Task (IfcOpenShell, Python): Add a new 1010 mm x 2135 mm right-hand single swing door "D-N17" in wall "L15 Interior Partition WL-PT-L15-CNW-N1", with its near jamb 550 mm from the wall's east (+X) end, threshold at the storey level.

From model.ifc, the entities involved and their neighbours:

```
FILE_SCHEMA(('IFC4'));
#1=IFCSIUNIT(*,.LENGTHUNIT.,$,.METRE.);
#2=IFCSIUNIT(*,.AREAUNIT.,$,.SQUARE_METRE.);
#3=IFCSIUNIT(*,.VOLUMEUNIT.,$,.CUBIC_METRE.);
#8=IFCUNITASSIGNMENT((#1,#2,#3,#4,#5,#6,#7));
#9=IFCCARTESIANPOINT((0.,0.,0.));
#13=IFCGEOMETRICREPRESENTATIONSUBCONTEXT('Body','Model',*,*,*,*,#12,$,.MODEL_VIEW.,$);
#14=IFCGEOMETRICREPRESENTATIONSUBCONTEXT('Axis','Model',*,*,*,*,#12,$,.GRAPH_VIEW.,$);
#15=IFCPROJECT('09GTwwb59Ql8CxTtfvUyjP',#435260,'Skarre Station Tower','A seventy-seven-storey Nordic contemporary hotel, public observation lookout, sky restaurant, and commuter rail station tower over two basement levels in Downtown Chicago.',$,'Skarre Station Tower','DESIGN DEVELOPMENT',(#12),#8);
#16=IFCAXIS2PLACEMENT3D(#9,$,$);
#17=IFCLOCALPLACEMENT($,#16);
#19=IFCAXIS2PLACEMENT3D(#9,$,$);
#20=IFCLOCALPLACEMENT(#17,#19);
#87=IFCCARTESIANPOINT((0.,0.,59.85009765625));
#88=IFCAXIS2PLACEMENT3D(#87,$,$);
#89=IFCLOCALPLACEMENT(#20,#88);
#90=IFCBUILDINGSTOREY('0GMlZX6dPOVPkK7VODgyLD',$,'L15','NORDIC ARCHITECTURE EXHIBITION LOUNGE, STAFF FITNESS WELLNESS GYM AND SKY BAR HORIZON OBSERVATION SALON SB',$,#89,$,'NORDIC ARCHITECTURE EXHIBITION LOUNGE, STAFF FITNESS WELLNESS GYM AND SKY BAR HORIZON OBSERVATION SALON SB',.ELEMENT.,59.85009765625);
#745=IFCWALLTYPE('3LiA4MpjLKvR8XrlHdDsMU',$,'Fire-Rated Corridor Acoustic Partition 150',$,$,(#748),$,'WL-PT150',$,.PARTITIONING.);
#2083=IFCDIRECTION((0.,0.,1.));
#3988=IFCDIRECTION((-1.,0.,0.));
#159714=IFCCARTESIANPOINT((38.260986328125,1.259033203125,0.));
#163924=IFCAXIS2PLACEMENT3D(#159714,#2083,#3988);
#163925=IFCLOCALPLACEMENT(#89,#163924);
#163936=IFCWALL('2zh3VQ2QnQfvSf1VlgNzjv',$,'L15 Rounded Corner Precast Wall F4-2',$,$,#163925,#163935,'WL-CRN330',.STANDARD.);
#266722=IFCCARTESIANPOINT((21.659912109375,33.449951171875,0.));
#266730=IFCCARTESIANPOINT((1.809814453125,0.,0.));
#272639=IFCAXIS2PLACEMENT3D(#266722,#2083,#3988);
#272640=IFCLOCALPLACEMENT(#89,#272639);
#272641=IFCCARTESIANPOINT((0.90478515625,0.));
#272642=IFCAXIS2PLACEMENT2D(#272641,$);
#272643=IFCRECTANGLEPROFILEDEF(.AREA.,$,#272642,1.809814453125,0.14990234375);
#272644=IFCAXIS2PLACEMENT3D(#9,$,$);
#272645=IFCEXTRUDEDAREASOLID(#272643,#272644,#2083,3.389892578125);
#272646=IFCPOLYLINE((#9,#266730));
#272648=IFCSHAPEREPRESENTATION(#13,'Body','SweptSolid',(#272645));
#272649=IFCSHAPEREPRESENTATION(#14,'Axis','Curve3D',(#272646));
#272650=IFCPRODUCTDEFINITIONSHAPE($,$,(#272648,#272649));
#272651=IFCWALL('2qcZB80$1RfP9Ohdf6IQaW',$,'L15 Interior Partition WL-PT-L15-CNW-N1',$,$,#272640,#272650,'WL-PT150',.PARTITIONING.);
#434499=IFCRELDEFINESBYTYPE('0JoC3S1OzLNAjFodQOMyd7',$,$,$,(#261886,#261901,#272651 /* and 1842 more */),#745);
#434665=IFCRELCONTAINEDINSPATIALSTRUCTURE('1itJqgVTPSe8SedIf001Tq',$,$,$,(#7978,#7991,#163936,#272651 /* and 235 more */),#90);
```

```python
import numpy as np
import ifcopenshell
import ifcopenshell.api.feature
import ifcopenshell.api.geometry
import ifcopenshell.api.root
import ifcopenshell.api.spatial
import ifcopenshell.geom
import ifcopenshell.util.element
import ifcopenshell.util.placement
import ifcopenshell.util.representation
import ifcopenshell.util.shape
import ifcopenshell.util.unit

model = ifcopenshell.open("model.ifc")
unit_scale = ifcopenshell.util.unit.calculate_unit_scale(model)
settings = ifcopenshell.geom.settings()


def volume(element):
    """Net volume in cubic metres, openings subtracted."""
    shape = ifcopenshell.geom.create_shape(settings, element)
    return ifcopenshell.util.shape.get_volume(shape.geometry)


wall = model.by_guid("2qcZB80$1RfP9Ohdf6IQaW")
storey = ifcopenshell.util.element.get_container(wall, ifc_class="IfcBuildingStorey")
context = ifcopenshell.util.representation.get_context(model, "Model", "Body", "MODEL_VIEW")
before = volume(wall)

width, height, from_end, sill = 1.01, 2.135, 0.55, 0.0  # metres

# The wall runs along its own X axis, and the end named is its -X end.
wall_shape = ifcopenshell.geom.create_shape(settings, wall)
x, y, z = ifcopenshell.util.shape.get_vertices(wall_shape.geometry).T
start = x.min() + from_end
face, thickness = float(y.min()), float(y.max() - y.min())
wall_matrix = ifcopenshell.util.placement.get_local_placement(wall.ObjectPlacement)
level = ifcopenshell.util.placement.get_local_placement(storey.ObjectPlacement)[2, 3]


def in_wall(x, y):
    """Placement at x, y metres in the wall's axes, at sill height."""
    matrix = wall_matrix.copy()
    matrix[:, 3] = wall_matrix @ np.array([x / unit_scale, y / unit_scale, 0.0, 1.0])
    matrix[2, 3] = level + sill / unit_scale
    return matrix


# Opening: a box that overshoots both wall faces by 50 mm.
opening = ifcopenshell.api.root.create_entity(model, ifc_class="IfcOpeningElement", predefined_type="OPENING")
box = ifcopenshell.api.geometry.add_wall_representation(
    model, context=context, length=width, height=height, thickness=thickness + 0.1
)
ifcopenshell.api.geometry.assign_representation(model, product=opening, representation=box)
ifcopenshell.api.geometry.edit_object_placement(model, product=opening, matrix=in_wall(start, face - 0.05), is_si=False)
ifcopenshell.api.feature.add_feature(model, feature=opening, element=wall)

door = ifcopenshell.api.root.create_entity(model, ifc_class="IfcDoor", name="D-N17", predefined_type="DOOR")
door.OverallWidth, door.OverallHeight = width / unit_scale, height / unit_scale
door.OperationType = "SINGLE_SWING_RIGHT"
body = ifcopenshell.api.geometry.add_door_representation(
    model,
    context=context,
    overall_width=door.OverallWidth,
    overall_height=door.OverallHeight,
    operation_type="SINGLE_SWING_RIGHT",
    lining_properties={"LiningDepth": thickness / unit_scale, "ThresholdDepth": thickness / unit_scale},
)
ifcopenshell.api.geometry.assign_representation(model, product=door, representation=body)
ifcopenshell.api.spatial.assign_container(model, products=[door], relating_structure=storey)
ifcopenshell.api.feature.add_filling(model, opening=opening, element=door)

# The lining spans the wall, so the door starts at the wall face.
ifcopenshell.api.geometry.edit_object_placement(model, product=door, matrix=in_wall(start, face), is_si=False)

after = volume(wall)

print(f"wall volume {before:.3f} -> {after:.3f} m3")

model.write("model_rev.ifc")
```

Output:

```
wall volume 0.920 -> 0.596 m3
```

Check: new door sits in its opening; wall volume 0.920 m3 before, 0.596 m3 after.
